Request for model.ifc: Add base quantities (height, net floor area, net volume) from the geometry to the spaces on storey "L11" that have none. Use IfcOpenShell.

First a look at what the model holds.

```python
import ifcopenshell
import ifcopenshell.util.element
import ifcopenshell.util.unit

model = ifcopenshell.open("model.ifc")
print(model.schema)
for unit_type in ("LENGTHUNIT", "AREAUNIT", "VOLUMEUNIT"):
    print(unit_type, ifcopenshell.util.unit.calculate_unit_scale(model, unit_type))
storey = next(s for s in model.by_type("IfcBuildingStorey") if s.Name == "L11")
spaces = [e for e in ifcopenshell.util.element.get_decomposition(storey) if e.is_a("IfcSpace")]
for e in sorted(spaces, key=lambda e: e.id()):
    print(e.id(), e.is_a(), e.Name, list(ifcopenshell.util.element.get_psets(e, qtos_only=True)), sep=" | ")
```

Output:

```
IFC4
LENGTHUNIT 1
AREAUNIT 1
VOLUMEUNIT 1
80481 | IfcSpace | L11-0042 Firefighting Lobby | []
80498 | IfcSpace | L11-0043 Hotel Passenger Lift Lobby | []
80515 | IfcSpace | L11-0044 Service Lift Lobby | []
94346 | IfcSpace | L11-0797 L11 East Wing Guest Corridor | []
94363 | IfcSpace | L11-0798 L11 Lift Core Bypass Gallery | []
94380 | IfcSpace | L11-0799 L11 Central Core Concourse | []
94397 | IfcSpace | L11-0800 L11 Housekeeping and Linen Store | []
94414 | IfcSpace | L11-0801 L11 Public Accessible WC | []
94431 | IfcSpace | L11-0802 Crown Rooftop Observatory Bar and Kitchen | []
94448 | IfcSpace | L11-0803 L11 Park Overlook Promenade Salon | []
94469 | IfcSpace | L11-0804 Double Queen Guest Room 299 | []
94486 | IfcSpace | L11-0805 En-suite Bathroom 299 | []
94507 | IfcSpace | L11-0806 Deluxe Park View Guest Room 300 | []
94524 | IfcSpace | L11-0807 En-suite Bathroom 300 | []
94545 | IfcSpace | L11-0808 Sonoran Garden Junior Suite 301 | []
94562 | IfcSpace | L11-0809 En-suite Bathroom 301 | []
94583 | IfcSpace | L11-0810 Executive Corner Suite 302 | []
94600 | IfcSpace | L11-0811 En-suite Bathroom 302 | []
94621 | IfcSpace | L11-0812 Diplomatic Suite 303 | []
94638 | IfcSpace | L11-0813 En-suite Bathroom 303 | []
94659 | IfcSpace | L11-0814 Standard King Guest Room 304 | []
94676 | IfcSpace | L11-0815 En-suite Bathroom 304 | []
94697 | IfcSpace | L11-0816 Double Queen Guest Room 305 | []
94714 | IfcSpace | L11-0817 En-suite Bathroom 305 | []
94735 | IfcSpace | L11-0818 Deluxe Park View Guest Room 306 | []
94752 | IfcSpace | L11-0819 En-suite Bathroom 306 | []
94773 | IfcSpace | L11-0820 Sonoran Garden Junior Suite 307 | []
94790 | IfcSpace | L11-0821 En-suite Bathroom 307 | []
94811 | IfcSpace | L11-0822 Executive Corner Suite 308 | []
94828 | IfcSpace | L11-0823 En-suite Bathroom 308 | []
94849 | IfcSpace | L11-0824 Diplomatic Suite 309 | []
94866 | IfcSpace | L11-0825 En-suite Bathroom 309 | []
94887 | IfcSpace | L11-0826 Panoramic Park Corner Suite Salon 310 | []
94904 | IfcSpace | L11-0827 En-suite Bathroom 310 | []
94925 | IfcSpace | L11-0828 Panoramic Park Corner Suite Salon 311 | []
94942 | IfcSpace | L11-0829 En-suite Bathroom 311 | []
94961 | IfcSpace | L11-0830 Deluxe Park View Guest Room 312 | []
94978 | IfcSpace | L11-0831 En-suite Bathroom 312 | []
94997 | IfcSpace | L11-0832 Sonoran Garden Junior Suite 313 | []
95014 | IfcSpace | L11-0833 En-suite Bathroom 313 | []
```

```python
import ifcopenshell
import ifcopenshell.api.pset
import ifcopenshell.geom
import ifcopenshell.util.element
import ifcopenshell.util.shape
import ifcopenshell.util.unit

model = ifcopenshell.open("model.ifc")
unit_scale = ifcopenshell.util.unit.calculate_unit_scale(model)
area_scale = ifcopenshell.util.unit.calculate_unit_scale(model, "AREAUNIT")
volume_scale = ifcopenshell.util.unit.calculate_unit_scale(model, "VOLUMEUNIT")
settings = ifcopenshell.geom.settings()

storey = next(s for s in model.by_type("IfcBuildingStorey") if s.Name == "L11")
spaces = [e for e in ifcopenshell.util.element.get_decomposition(storey) if e.is_a("IfcSpace")]

for e in sorted(spaces, key=lambda e: e.id()):
    if ifcopenshell.util.element.get_psets(e, qtos_only=True, should_inherit=False):
        continue
    # Geometry comes back in metres, in the element's own axes.
    shape = ifcopenshell.geom.create_shape(settings, e)
    values = {
        "Height": ifcopenshell.util.shape.get_z(shape.geometry) / unit_scale,
        "NetFloorArea": ifcopenshell.util.shape.get_footprint_area(shape.geometry) / area_scale,
        "NetVolume": ifcopenshell.util.shape.get_volume(shape.geometry) / volume_scale,
    }
    qto = ifcopenshell.api.pset.add_qto(model, product=e, name="Qto_SpaceBaseQuantities")
    ifcopenshell.api.pset.edit_qto(model, qto=qto, properties=values)
    print(e.id(), {k: round(v, 3) for k, v in values.items()})

model.write("model_v2.ifc")
```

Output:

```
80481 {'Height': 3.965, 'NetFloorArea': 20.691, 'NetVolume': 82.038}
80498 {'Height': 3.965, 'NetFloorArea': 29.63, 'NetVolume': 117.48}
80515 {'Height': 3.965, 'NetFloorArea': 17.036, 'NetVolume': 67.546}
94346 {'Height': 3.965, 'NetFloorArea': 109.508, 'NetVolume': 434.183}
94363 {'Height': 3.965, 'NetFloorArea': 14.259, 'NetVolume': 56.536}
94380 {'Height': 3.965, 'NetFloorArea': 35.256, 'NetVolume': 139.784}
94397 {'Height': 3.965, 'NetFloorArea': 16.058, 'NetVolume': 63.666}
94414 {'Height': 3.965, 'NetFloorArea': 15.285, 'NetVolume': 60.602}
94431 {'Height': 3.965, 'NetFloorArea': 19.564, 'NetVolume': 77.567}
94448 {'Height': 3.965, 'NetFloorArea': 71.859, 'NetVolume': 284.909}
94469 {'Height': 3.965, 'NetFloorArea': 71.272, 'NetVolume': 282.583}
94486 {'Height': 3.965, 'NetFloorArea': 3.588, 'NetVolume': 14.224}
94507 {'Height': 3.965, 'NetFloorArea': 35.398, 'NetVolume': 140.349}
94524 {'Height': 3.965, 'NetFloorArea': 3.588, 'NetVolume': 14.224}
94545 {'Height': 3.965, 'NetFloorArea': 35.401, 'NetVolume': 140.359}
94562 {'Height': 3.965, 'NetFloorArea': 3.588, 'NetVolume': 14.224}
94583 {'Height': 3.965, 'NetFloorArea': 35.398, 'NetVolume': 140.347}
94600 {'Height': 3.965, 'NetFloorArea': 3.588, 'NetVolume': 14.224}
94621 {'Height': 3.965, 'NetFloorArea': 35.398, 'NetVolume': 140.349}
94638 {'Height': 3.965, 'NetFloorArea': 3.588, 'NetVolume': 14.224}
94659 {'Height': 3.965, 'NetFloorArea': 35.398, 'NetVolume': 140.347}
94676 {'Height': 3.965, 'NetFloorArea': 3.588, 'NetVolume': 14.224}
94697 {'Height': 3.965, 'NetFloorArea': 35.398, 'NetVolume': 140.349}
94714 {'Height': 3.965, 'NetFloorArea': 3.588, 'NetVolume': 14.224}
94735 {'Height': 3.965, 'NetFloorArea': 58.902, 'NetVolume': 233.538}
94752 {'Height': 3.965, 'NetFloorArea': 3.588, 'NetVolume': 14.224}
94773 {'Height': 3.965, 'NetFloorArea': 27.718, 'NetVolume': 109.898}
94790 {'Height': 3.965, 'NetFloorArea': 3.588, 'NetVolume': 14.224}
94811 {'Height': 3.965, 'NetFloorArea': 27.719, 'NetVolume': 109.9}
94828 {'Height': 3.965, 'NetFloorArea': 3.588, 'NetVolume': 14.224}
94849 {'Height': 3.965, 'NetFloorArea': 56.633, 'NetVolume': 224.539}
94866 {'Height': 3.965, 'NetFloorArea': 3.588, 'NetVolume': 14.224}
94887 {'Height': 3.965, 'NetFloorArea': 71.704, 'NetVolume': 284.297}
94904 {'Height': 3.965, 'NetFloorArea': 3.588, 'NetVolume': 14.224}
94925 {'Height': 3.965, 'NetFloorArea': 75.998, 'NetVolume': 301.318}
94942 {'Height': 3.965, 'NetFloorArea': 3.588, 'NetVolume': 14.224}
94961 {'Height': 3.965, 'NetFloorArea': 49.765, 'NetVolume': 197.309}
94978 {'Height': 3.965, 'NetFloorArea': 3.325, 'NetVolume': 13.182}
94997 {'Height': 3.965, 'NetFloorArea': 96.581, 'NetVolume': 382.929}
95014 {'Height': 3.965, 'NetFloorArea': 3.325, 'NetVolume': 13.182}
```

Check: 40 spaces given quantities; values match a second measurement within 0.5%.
